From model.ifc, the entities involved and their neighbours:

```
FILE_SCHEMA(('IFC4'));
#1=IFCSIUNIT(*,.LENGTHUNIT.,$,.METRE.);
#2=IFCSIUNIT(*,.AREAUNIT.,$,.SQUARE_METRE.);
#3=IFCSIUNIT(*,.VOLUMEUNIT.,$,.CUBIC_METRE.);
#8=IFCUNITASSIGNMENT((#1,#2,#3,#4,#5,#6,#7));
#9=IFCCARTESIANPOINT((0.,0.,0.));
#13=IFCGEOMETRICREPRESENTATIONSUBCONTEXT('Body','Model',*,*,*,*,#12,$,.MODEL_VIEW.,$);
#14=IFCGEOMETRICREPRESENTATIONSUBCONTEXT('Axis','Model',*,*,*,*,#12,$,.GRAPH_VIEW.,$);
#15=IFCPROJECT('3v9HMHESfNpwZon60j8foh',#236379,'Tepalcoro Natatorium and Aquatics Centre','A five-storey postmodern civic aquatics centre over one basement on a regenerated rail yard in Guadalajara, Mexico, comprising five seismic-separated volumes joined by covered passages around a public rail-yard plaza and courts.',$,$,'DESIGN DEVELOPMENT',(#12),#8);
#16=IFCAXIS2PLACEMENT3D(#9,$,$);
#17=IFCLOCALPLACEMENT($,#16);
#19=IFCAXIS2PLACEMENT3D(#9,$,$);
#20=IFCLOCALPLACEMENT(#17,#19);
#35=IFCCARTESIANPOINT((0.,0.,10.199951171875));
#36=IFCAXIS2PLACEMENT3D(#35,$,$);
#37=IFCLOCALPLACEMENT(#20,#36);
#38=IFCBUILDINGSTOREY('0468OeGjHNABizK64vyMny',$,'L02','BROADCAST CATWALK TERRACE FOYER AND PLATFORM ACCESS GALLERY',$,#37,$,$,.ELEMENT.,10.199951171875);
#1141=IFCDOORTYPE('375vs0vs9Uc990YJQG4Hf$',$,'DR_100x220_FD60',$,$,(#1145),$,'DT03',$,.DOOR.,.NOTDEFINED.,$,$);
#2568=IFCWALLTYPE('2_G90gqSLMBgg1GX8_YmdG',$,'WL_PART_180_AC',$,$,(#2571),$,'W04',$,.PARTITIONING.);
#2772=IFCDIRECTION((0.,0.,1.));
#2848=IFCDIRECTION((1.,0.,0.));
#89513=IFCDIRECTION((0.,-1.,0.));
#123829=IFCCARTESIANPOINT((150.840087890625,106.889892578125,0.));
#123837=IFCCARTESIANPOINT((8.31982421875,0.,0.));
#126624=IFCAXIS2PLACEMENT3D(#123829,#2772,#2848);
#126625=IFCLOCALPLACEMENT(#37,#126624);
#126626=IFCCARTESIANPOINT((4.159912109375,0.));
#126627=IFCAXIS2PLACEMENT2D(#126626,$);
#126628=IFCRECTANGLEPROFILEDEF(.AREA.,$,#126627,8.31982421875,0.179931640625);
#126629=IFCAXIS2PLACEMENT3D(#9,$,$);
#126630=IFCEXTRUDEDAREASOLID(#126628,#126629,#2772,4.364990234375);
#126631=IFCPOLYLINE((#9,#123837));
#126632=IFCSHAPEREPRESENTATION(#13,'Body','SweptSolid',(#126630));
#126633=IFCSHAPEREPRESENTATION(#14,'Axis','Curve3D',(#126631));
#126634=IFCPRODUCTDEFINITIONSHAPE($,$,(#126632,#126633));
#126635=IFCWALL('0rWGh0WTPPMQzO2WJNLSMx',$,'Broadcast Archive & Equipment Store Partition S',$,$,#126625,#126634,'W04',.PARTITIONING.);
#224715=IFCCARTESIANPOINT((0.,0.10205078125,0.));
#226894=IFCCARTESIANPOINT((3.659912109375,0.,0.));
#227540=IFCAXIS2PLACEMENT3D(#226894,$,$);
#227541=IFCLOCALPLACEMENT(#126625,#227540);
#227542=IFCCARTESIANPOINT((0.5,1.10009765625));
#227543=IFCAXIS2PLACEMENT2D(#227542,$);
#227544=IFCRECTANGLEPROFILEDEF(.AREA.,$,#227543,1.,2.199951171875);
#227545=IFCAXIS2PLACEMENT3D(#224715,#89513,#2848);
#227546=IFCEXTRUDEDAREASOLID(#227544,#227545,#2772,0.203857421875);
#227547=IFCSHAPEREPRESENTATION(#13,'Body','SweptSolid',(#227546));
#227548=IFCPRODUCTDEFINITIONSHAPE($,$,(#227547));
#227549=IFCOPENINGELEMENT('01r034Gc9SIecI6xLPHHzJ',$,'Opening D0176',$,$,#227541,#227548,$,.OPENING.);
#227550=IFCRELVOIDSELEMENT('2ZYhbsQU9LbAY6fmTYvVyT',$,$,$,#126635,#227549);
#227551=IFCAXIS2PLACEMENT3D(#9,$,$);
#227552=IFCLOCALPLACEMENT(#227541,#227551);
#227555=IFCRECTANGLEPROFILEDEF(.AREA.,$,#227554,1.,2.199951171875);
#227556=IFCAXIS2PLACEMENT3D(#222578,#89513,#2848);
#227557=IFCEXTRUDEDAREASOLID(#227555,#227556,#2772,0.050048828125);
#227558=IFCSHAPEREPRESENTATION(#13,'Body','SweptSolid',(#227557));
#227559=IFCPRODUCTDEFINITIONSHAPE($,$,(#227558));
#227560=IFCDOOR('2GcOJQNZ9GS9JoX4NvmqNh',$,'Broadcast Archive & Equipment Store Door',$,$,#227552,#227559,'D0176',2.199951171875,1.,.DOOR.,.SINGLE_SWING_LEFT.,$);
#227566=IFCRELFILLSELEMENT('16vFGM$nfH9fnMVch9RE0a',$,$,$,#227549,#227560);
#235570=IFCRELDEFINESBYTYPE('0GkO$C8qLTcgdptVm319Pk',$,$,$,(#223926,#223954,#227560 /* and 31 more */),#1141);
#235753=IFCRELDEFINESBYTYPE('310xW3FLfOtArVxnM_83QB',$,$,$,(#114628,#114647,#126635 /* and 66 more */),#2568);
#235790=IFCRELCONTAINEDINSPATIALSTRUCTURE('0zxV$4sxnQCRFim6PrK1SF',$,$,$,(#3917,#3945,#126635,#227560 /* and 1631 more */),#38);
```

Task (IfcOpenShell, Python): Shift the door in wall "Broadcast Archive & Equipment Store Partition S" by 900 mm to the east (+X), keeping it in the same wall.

```python
import ifcopenshell
import ifcopenshell.api.geometry
import ifcopenshell.util.placement
import ifcopenshell.util.unit

model = ifcopenshell.open("model.ifc")
unit_scale = ifcopenshell.util.unit.calculate_unit_scale(model)

door = model.by_guid("2GcOJQNZ9GS9JoX4NvmqNh")
opening = door.FillsVoids[0].RelatingOpeningElement
wall = opening.VoidsElements[0].RelatingBuildingElement

wall_matrix = ifcopenshell.util.placement.get_local_placement(wall.ObjectPlacement)
shift = wall_matrix[:3, 0] * 0.9 / unit_scale
before = ifcopenshell.util.placement.get_local_placement(door.ObjectPlacement)[:3, 3].copy()

# The door is placed relative to its opening, so it follows when the opening moves.
matrix = ifcopenshell.util.placement.get_local_placement(opening.ObjectPlacement)
matrix[:3, 3] += shift
ifcopenshell.api.geometry.edit_object_placement(
    model, product=opening, matrix=matrix, is_si=False, should_transform_children=True
)

after = ifcopenshell.util.placement.get_local_placement(door.ObjectPlacement)[:3, 3]
print("door moved by", (after - before).round(3) + 0.0)

model.write("model-out.ifc")
```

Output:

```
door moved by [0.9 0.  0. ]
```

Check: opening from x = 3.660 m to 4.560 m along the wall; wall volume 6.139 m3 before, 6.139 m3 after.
